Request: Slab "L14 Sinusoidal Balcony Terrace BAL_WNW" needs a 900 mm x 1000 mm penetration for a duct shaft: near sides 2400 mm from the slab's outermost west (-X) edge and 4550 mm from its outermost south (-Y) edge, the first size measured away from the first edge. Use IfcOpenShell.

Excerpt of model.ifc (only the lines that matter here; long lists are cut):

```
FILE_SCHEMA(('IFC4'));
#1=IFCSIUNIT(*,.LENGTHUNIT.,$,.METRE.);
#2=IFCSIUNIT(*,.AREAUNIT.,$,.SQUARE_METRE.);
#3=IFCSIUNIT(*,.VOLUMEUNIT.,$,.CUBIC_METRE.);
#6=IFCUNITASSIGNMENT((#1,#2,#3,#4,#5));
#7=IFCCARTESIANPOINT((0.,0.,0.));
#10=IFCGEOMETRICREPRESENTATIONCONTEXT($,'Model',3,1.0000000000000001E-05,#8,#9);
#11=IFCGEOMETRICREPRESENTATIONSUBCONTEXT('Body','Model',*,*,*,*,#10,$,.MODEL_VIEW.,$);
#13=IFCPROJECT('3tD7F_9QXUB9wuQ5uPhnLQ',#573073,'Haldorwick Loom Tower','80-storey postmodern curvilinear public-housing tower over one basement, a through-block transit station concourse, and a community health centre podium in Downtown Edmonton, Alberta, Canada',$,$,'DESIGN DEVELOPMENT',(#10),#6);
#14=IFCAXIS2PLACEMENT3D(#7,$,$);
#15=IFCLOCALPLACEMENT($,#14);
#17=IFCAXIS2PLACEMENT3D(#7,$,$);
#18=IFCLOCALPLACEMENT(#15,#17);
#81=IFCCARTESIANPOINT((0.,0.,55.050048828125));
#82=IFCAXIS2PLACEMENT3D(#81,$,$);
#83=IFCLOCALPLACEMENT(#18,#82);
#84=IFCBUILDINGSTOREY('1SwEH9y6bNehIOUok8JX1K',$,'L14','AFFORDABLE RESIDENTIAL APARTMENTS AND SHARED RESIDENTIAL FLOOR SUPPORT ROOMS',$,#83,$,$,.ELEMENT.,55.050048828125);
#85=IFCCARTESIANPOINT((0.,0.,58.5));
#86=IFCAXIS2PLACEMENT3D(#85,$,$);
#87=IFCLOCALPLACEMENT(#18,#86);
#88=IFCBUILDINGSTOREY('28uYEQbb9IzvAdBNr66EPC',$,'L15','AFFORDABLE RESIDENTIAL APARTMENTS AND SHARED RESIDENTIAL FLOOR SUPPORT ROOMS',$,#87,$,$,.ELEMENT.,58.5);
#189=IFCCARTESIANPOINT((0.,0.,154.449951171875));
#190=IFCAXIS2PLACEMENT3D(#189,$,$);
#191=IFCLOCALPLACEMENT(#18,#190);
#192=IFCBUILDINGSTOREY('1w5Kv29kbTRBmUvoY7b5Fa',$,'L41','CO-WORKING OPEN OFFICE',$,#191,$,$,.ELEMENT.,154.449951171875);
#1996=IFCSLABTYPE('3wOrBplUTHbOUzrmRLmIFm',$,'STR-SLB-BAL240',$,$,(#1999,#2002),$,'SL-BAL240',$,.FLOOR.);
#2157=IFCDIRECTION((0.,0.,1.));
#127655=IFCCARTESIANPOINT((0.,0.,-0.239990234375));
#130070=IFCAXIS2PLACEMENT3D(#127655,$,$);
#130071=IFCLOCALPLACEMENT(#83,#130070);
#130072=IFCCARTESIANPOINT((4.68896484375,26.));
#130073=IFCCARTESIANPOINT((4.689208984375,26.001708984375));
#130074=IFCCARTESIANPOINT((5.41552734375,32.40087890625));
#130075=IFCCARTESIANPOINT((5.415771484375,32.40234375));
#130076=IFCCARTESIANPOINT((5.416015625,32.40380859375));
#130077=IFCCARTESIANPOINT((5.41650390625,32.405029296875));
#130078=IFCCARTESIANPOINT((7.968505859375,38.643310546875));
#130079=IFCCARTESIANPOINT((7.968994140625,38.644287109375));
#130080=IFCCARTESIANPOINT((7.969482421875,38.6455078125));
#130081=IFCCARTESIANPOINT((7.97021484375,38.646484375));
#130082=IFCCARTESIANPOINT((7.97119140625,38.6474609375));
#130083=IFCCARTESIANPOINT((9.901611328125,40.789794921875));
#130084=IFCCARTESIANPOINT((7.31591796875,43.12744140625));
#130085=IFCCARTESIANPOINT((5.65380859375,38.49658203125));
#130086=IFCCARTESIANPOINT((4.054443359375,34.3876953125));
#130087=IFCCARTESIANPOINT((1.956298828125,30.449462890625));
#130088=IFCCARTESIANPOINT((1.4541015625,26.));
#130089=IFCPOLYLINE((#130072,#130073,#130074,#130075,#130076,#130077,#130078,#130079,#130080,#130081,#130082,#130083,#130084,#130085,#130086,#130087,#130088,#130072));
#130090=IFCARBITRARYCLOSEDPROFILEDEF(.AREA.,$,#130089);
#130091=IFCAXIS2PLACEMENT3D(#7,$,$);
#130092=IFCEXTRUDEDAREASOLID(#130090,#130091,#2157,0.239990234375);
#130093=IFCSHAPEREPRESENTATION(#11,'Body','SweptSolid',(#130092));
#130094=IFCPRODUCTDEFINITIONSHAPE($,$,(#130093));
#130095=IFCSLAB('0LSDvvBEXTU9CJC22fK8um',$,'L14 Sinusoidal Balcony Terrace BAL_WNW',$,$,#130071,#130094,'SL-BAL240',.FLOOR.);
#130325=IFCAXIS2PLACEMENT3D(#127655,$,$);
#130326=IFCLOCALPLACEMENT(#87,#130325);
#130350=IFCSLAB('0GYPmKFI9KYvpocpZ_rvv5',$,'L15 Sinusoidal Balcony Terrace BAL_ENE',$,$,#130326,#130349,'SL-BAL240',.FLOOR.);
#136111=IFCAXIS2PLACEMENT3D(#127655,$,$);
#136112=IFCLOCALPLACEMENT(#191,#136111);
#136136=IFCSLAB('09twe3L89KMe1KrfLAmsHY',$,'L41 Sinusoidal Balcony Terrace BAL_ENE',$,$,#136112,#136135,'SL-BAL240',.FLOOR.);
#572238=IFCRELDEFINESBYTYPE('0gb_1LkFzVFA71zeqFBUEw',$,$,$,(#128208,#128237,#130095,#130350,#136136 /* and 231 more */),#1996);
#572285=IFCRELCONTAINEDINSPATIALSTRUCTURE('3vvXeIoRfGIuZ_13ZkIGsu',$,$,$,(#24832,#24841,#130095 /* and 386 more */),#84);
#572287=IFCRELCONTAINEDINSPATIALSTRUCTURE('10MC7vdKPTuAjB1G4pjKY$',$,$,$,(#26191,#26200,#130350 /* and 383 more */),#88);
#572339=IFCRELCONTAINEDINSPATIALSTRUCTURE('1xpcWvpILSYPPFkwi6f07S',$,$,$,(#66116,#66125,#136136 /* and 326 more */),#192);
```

```python
import numpy as np
import ifcopenshell
import ifcopenshell.api.feature
import ifcopenshell.api.geometry
import ifcopenshell.api.root
import ifcopenshell.geom
import ifcopenshell.util.placement
import ifcopenshell.util.representation
import ifcopenshell.util.shape
import ifcopenshell.util.unit

model = ifcopenshell.open("model.ifc")
unit_scale = ifcopenshell.util.unit.calculate_unit_scale(model)
settings = ifcopenshell.geom.settings()


def volume(element):
    """Net volume in cubic metres, openings subtracted."""
    shape = ifcopenshell.geom.create_shape(settings, element)
    return ifcopenshell.util.shape.get_volume(shape.geometry)


slab = model.by_guid("0LSDvvBEXTU9CJC22fK8um")
before = volume(slab)

# Extent in the slab's own axes, in metres. The edges named are its -X and -Y sides.
slab_shape = ifcopenshell.geom.create_shape(settings, slab)
vertices = ifcopenshell.util.shape.get_vertices(slab_shape.geometry)
x_min, y_min, bottom = vertices.min(axis=0)
top = vertices[:, 2].max()

opening = ifcopenshell.api.root.create_entity(model, ifc_class="IfcOpeningElement", name="Duct shaft opening", predefined_type="OPENING")
context = ifcopenshell.util.representation.get_context(model, "Model", "Body", "MODEL_VIEW")
width, depth = 0.9, 1
outline = [(0.0, 0.0), (width, 0.0), (width, depth), (0.0, depth), (0.0, 0.0)]
# Overshoot both faces by 50 mm so the cut is clean.
shape = ifcopenshell.api.geometry.add_slab_representation(
    model, context=context, depth=top - bottom + 0.1, polyline=outline
)
ifcopenshell.api.geometry.assign_representation(model, product=opening, representation=shape)

matrix = ifcopenshell.util.placement.get_local_placement(slab.ObjectPlacement)
matrix[:, 3] = matrix @ np.append(np.array([x_min + 2.4, y_min + 4.55, bottom - 0.05]) / unit_scale, 1.0)
ifcopenshell.api.geometry.edit_object_placement(model, product=opening, matrix=matrix, is_si=False)
ifcopenshell.api.feature.add_feature(model, feature=opening, element=slab)

after = volume(slab)

print(f"slab volume {before:.3f} -> {after:.3f} m3")

model.write("model_edited.ifc")
```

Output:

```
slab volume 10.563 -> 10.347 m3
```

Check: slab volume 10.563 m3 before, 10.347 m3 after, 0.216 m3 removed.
